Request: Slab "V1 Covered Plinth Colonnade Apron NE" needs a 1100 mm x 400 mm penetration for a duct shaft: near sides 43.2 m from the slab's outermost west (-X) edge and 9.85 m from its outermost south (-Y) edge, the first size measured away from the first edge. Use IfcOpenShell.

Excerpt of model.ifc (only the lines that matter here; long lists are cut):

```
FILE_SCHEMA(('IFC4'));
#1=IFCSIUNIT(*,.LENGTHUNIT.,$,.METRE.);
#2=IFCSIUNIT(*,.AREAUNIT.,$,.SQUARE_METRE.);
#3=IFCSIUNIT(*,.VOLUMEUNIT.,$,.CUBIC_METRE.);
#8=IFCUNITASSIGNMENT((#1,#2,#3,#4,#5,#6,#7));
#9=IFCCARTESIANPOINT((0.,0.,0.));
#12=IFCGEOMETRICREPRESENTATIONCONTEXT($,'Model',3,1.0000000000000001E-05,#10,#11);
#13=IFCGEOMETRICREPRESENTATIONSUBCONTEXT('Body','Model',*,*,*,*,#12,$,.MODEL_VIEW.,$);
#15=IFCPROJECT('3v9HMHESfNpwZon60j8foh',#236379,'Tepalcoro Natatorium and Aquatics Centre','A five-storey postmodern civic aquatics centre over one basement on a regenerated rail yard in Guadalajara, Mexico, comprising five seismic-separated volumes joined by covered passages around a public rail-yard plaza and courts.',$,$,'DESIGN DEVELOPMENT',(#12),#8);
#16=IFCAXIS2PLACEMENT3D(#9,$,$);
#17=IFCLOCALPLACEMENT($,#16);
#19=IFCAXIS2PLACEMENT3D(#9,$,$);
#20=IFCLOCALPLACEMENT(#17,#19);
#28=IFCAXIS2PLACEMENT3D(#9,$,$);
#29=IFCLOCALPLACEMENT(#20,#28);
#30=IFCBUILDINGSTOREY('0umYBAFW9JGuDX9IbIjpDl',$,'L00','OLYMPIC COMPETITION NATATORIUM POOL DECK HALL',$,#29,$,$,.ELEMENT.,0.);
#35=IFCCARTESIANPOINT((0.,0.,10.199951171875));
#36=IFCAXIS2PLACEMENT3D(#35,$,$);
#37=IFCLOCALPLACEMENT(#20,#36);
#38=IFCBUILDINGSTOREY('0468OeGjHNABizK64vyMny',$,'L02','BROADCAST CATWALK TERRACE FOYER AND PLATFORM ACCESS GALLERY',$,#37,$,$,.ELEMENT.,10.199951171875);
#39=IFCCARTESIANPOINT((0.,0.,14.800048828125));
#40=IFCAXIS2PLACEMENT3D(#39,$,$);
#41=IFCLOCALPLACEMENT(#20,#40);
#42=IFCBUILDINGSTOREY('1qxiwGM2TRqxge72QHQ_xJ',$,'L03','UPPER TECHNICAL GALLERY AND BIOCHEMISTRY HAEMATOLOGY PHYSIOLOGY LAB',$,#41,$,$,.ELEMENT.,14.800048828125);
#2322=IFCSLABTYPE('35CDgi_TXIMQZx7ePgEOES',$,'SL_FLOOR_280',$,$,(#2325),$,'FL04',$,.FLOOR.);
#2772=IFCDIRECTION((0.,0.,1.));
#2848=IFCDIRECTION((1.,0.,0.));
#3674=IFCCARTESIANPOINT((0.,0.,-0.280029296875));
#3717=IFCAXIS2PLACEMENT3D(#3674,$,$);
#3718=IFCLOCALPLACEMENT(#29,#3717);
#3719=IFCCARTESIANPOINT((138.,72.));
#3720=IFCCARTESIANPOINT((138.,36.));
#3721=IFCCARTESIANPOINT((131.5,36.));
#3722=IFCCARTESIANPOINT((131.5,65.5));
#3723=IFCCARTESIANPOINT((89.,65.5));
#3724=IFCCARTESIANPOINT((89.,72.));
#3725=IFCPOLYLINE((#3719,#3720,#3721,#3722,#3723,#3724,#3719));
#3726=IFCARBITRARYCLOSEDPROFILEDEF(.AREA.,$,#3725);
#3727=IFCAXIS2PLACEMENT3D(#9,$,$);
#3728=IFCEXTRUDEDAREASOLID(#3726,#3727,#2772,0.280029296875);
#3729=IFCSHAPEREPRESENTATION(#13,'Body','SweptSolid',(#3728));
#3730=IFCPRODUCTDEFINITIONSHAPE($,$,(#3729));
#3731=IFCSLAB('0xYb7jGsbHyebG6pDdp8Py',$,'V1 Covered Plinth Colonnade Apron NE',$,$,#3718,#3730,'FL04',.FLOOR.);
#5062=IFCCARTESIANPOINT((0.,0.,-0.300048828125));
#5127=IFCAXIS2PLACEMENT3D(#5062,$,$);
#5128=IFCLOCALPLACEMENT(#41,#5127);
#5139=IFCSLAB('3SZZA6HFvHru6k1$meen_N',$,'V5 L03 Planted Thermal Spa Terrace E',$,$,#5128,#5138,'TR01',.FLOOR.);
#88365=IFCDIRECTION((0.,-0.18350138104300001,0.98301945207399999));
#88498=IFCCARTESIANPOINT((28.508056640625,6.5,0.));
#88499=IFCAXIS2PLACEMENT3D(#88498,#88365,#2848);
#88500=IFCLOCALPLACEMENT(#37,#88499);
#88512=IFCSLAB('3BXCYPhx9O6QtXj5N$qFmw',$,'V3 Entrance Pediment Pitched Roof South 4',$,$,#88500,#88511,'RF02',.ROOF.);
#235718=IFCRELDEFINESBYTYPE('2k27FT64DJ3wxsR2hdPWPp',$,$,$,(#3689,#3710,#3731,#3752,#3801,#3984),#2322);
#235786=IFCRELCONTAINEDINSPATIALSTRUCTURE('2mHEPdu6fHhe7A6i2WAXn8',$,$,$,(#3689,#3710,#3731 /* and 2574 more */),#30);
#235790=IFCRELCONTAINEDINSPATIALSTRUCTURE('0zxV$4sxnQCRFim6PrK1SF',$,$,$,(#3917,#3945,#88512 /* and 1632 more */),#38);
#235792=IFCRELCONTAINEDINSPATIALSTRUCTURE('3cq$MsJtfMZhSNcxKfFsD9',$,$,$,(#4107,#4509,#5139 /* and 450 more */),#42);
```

```python
import numpy as np
import ifcopenshell
import ifcopenshell.api.feature
import ifcopenshell.api.geometry
import ifcopenshell.api.root
import ifcopenshell.geom
import ifcopenshell.util.placement
import ifcopenshell.util.representation
import ifcopenshell.util.shape
import ifcopenshell.util.unit

model = ifcopenshell.open("model.ifc")
unit_scale = ifcopenshell.util.unit.calculate_unit_scale(model)
settings = ifcopenshell.geom.settings()


def volume(element):
    """Net volume in cubic metres, openings subtracted."""
    shape = ifcopenshell.geom.create_shape(settings, element)
    return ifcopenshell.util.shape.get_volume(shape.geometry)


slab = model.by_guid("0xYb7jGsbHyebG6pDdp8Py")
before = volume(slab)

# Extent in the slab's own axes, in metres. The edges named are its -X and -Y sides.
slab_shape = ifcopenshell.geom.create_shape(settings, slab)
vertices = ifcopenshell.util.shape.get_vertices(slab_shape.geometry)
x_min, y_min, bottom = vertices.min(axis=0)
top = vertices[:, 2].max()

opening = ifcopenshell.api.root.create_entity(model, ifc_class="IfcOpeningElement", name="Duct shaft opening", predefined_type="OPENING")
context = ifcopenshell.util.representation.get_context(model, "Model", "Body", "MODEL_VIEW")
width, depth = 1.1, 0.4
outline = [(0.0, 0.0), (width, 0.0), (width, depth), (0.0, depth), (0.0, 0.0)]
# Overshoot both faces by 50 mm so the cut is clean.
shape = ifcopenshell.api.geometry.add_slab_representation(
    model, context=context, depth=top - bottom + 0.1, polyline=outline
)
ifcopenshell.api.geometry.assign_representation(model, product=opening, representation=shape)

matrix = ifcopenshell.util.placement.get_local_placement(slab.ObjectPlacement)
matrix[:, 3] = matrix @ np.append(np.array([x_min + 43.2, y_min + 9.85, bottom - 0.05]) / unit_scale, 1.0)
ifcopenshell.api.geometry.edit_object_placement(model, product=opening, matrix=matrix, is_si=False)
ifcopenshell.api.feature.add_feature(model, feature=opening, element=slab)

after = volume(slab)

print(f"slab volume {before:.3f} -> {after:.3f} m3")

model.write("model_v2.ifc")
```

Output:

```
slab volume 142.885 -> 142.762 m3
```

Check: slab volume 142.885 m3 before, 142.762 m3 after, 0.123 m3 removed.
